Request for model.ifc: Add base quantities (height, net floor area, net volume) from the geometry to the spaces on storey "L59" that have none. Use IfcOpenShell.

First a look at what the model holds.

```python
import ifcopenshell
import ifcopenshell.util.element
import ifcopenshell.util.unit

model = ifcopenshell.open("model.ifc")
print(model.schema)
for unit_type in ("LENGTHUNIT", "AREAUNIT", "VOLUMEUNIT"):
    print(unit_type, ifcopenshell.util.unit.calculate_unit_scale(model, unit_type))
storey = next(s for s in model.by_type("IfcBuildingStorey") if s.Name == "L59")
spaces = [e for e in ifcopenshell.util.element.get_decomposition(storey) if e.is_a("IfcSpace")]
for e in sorted(spaces, key=lambda e: e.id()):
    print(e.id(), e.is_a(), e.Name, list(ifcopenshell.util.element.get_psets(e, qtos_only=True)), sep=" | ")
```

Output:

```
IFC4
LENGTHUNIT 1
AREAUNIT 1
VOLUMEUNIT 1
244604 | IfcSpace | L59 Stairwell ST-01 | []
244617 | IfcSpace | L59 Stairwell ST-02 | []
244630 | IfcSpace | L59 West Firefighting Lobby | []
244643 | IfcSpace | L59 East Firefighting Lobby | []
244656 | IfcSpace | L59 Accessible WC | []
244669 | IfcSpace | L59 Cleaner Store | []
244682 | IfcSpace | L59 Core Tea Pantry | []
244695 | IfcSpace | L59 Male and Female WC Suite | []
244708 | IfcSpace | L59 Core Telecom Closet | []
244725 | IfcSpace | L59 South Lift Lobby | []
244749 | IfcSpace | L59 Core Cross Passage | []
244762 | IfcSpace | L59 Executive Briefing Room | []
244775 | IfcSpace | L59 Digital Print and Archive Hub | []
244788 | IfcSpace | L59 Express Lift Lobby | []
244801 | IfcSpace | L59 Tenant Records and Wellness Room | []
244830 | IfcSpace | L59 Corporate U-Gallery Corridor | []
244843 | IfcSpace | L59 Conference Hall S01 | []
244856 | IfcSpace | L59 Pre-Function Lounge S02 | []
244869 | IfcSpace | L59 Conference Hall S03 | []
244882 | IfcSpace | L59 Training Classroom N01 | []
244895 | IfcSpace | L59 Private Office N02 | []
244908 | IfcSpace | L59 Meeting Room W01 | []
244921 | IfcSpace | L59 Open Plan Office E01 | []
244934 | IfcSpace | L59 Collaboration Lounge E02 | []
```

```python
import ifcopenshell
import ifcopenshell.api.pset
import ifcopenshell.geom
import ifcopenshell.util.element
import ifcopenshell.util.shape
import ifcopenshell.util.unit

model = ifcopenshell.open("model.ifc")
unit_scale = ifcopenshell.util.unit.calculate_unit_scale(model)
area_scale = ifcopenshell.util.unit.calculate_unit_scale(model, "AREAUNIT")
volume_scale = ifcopenshell.util.unit.calculate_unit_scale(model, "VOLUMEUNIT")
settings = ifcopenshell.geom.settings()

storey = next(s for s in model.by_type("IfcBuildingStorey") if s.Name == "L59")
spaces = [e for e in ifcopenshell.util.element.get_decomposition(storey) if e.is_a("IfcSpace")]

for e in sorted(spaces, key=lambda e: e.id()):
    if ifcopenshell.util.element.get_psets(e, qtos_only=True, should_inherit=False):
        continue
    # Geometry comes back in metres, in the element's own axes.
    shape = ifcopenshell.geom.create_shape(settings, e)
    values = {
        "Height": ifcopenshell.util.shape.get_z(shape.geometry) / unit_scale,
        "NetFloorArea": ifcopenshell.util.shape.get_footprint_area(shape.geometry) / area_scale,
        "NetVolume": ifcopenshell.util.shape.get_volume(shape.geometry) / volume_scale,
    }
    qto = ifcopenshell.api.pset.add_qto(model, product=e, name="Qto_SpaceBaseQuantities")
    ifcopenshell.api.pset.edit_qto(model, qto=qto, properties=values)
    print(e.id(), {k: round(v, 3) for k, v in values.items()})

model.write("model_v2.ifc")
```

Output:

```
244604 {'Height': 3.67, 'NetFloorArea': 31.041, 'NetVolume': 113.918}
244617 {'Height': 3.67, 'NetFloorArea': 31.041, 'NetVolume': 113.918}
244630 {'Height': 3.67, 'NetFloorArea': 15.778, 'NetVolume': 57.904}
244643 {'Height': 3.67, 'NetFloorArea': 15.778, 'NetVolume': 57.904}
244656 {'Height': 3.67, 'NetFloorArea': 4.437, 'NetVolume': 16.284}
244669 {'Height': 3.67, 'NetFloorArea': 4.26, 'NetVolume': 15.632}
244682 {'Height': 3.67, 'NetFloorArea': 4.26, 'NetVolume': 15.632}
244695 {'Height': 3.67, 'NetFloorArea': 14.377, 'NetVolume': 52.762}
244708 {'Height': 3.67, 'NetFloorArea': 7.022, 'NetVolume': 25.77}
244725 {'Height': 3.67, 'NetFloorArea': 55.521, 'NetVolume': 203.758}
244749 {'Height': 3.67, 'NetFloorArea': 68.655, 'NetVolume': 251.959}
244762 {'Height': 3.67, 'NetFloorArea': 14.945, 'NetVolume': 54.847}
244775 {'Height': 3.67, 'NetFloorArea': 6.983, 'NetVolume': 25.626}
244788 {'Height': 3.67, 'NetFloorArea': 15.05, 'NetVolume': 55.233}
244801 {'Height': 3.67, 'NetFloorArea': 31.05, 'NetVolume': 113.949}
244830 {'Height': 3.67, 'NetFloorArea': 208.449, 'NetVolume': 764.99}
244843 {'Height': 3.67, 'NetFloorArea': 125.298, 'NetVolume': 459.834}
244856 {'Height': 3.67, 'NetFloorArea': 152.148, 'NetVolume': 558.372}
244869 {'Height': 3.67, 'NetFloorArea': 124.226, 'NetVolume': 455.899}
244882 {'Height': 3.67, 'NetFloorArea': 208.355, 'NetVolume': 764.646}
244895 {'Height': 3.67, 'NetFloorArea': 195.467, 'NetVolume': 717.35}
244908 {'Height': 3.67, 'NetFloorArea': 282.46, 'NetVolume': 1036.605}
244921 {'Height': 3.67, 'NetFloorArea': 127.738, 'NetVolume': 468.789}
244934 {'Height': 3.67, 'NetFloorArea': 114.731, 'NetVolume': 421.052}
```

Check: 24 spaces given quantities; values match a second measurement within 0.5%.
